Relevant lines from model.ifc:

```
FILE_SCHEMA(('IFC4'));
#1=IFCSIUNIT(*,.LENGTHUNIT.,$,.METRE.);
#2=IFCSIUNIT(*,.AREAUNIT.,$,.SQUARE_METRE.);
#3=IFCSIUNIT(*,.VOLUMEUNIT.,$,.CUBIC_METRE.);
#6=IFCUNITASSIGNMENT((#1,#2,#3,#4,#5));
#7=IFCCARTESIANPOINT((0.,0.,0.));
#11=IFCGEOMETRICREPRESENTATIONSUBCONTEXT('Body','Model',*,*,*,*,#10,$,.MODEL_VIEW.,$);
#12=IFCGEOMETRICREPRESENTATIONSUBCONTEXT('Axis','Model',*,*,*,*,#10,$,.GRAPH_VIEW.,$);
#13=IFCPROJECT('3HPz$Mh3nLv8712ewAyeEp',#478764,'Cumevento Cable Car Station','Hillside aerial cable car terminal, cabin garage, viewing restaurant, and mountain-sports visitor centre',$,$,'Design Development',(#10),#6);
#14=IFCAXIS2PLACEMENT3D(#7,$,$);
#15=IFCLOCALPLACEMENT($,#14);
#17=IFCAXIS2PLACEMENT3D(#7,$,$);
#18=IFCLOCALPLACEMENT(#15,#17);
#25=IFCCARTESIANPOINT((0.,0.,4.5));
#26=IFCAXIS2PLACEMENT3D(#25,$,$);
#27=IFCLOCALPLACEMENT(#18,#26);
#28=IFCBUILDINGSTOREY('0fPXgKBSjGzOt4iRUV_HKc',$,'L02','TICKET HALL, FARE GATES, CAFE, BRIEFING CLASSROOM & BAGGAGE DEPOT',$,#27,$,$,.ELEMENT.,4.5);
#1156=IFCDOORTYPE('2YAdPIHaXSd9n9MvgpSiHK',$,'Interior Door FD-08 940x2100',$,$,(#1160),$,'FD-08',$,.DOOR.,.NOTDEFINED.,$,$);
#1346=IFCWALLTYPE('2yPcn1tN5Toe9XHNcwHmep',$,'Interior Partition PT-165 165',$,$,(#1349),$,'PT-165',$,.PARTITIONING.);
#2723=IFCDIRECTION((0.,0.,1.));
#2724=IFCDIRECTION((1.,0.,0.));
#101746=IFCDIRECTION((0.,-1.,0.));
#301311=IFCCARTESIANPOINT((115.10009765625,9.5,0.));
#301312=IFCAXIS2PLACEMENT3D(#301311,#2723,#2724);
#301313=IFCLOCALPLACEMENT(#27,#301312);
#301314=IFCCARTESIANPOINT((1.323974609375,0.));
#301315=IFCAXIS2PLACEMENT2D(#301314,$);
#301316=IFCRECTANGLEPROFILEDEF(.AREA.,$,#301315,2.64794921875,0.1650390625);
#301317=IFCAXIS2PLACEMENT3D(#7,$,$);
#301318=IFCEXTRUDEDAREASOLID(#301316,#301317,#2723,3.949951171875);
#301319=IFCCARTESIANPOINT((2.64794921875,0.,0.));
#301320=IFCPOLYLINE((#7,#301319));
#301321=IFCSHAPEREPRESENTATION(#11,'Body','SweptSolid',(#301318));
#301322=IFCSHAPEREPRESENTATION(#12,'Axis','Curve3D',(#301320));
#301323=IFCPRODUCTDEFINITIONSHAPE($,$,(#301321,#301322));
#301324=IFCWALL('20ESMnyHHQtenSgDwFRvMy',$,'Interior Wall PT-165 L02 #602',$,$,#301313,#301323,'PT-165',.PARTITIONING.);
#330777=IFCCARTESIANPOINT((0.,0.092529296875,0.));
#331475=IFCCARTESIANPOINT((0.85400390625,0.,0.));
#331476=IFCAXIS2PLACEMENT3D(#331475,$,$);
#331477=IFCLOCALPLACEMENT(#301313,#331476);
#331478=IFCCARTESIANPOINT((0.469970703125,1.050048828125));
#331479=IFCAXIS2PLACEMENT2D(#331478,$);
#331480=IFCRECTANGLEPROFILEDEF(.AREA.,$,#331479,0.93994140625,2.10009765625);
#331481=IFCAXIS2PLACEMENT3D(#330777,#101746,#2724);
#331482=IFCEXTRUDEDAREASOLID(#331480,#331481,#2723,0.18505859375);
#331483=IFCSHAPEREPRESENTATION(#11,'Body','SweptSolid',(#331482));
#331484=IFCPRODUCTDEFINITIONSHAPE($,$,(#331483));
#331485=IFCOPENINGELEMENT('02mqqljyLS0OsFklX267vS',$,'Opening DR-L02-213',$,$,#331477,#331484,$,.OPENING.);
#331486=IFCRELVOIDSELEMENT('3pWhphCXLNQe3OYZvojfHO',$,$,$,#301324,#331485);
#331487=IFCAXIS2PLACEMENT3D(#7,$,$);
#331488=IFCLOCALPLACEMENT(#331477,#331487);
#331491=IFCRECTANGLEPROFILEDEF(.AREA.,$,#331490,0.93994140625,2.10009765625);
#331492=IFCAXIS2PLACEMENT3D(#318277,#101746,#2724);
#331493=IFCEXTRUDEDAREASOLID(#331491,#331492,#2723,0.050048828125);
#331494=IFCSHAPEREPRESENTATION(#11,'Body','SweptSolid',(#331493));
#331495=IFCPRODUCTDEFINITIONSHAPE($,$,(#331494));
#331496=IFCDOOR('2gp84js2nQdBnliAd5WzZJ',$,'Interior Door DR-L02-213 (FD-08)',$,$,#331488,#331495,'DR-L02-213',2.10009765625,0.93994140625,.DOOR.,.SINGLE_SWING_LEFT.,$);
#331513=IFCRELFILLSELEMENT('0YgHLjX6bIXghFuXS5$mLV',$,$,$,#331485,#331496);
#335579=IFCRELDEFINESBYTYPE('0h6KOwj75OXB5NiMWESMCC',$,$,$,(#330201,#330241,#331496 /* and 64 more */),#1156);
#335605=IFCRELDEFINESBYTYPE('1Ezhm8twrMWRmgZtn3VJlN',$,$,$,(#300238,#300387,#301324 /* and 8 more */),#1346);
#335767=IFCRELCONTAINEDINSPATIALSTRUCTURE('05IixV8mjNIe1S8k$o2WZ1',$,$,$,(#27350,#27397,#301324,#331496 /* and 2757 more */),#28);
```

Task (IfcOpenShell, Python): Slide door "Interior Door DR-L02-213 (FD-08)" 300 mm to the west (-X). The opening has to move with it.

```python
import ifcopenshell
import ifcopenshell.api.geometry
import ifcopenshell.util.placement

model = ifcopenshell.open("model.ifc")

door = model.by_guid("2gp84js2nQdBnliAd5WzZJ")
opening = door.FillsVoids[0].RelatingOpeningElement
wall = opening.VoidsElements[0].RelatingBuildingElement

wall_matrix = ifcopenshell.util.placement.get_local_placement(wall.ObjectPlacement)
shift = wall_matrix[:3, 0] * -0.3
before = ifcopenshell.util.placement.get_local_placement(door.ObjectPlacement)[:3, 3].copy()

# The door is placed relative to its opening, so it follows when the opening moves.
matrix = ifcopenshell.util.placement.get_local_placement(opening.ObjectPlacement)
matrix[:3, 3] += shift
ifcopenshell.api.geometry.edit_object_placement(
    model, product=opening, matrix=matrix, is_si=False, should_transform_children=True
)

after = ifcopenshell.util.placement.get_local_placement(door.ObjectPlacement)[:3, 3]
print("door moved by", (after - before).round(3) + 0.0)

model.write("model-out.ifc")
```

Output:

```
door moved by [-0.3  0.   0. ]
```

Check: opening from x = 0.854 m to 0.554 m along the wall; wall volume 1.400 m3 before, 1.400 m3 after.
